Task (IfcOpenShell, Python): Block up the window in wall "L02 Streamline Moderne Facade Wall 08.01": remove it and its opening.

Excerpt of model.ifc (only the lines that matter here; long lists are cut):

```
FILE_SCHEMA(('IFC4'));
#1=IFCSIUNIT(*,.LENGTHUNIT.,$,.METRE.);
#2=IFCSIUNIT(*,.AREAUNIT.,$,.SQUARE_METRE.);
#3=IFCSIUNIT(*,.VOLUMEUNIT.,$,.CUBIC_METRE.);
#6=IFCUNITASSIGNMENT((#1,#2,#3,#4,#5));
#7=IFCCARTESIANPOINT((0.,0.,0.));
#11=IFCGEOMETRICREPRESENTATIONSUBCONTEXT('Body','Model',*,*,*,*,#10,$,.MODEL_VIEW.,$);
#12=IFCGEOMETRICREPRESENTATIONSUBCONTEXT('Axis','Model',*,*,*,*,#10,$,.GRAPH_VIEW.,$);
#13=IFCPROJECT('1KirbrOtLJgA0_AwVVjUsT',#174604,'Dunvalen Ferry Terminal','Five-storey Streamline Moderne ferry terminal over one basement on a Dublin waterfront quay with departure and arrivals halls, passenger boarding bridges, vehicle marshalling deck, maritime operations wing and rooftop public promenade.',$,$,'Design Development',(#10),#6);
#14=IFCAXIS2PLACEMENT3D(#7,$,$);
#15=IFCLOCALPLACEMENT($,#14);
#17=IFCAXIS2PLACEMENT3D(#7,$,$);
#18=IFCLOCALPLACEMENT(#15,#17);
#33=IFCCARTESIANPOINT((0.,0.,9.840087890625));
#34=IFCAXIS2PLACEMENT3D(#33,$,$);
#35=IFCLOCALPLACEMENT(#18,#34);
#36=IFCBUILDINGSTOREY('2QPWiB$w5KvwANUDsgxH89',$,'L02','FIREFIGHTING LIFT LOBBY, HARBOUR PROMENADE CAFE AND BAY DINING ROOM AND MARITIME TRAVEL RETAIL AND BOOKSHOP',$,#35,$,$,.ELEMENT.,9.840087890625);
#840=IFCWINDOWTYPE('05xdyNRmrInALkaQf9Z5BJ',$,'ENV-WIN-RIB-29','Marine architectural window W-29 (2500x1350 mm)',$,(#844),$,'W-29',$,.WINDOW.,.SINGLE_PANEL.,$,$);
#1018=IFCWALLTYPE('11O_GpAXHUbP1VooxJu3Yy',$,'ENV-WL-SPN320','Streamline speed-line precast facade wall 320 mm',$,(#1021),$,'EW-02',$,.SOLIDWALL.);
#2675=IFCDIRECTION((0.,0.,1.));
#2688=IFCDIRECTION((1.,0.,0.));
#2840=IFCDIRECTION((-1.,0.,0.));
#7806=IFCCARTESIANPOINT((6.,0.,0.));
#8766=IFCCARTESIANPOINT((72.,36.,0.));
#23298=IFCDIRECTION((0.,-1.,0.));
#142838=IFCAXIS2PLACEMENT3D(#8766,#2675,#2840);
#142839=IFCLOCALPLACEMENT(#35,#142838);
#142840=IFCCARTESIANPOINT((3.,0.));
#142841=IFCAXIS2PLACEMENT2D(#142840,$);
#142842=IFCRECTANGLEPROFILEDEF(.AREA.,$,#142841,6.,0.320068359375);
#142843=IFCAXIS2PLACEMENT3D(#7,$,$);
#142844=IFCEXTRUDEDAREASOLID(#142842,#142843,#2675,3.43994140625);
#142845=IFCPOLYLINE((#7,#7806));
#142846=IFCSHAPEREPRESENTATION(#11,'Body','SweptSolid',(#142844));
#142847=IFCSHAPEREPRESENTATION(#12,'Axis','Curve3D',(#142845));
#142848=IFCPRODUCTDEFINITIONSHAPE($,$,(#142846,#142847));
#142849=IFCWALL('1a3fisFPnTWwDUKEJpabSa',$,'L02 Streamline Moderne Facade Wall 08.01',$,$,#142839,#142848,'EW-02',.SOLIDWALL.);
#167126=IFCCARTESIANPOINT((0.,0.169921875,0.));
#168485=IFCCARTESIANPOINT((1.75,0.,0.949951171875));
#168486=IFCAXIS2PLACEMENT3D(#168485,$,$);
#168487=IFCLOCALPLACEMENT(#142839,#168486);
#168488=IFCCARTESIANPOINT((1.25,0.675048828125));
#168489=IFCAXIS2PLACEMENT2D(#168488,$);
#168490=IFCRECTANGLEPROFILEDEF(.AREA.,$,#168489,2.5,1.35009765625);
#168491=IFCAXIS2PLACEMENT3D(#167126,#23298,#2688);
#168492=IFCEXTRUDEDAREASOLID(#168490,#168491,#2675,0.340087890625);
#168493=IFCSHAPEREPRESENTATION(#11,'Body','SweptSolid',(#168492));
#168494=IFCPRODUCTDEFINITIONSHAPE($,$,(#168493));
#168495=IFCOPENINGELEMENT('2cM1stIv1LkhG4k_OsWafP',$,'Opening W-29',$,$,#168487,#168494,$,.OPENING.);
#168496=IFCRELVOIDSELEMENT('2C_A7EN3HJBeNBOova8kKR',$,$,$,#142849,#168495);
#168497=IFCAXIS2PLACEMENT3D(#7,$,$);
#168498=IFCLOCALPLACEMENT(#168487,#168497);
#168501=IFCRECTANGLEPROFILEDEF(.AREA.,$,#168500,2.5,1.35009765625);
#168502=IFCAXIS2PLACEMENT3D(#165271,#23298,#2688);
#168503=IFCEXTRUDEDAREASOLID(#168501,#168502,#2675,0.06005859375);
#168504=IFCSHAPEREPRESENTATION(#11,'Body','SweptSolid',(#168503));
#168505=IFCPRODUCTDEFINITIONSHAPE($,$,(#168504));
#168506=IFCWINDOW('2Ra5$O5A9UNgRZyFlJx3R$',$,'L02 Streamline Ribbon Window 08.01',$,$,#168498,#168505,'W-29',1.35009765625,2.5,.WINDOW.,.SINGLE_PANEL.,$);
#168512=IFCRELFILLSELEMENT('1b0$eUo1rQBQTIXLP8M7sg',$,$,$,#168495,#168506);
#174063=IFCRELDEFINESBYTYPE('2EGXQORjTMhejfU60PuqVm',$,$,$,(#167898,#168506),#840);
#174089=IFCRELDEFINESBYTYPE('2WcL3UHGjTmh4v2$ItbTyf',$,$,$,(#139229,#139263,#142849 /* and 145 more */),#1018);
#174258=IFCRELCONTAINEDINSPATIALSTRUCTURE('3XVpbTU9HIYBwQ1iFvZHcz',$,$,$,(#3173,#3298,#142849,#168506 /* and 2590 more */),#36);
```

```python
import ifcopenshell
import ifcopenshell.api.feature
import ifcopenshell.api.root
import ifcopenshell.geom
import ifcopenshell.util.shape

model = ifcopenshell.open("model.ifc")
settings = ifcopenshell.geom.settings()


def volume(element):
    """Net volume in cubic metres, openings subtracted."""
    shape = ifcopenshell.geom.create_shape(settings, element)
    return ifcopenshell.util.shape.get_volume(shape.geometry)


window = model.by_guid("2Ra5$O5A9UNgRZyFlJx3R$")
opening = window.FillsVoids[0].RelatingOpeningElement
wall = opening.VoidsElements[0].RelatingBuildingElement
before = volume(wall)

ifcopenshell.api.root.remove_product(model, product=window)
ifcopenshell.api.feature.remove_feature(model, feature=opening)

after = volume(wall)

print(f"wall volume {before:.3f} -> {after:.3f} m3")

model.write("model_rev.ifc")
```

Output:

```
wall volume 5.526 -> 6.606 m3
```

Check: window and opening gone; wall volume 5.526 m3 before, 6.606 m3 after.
